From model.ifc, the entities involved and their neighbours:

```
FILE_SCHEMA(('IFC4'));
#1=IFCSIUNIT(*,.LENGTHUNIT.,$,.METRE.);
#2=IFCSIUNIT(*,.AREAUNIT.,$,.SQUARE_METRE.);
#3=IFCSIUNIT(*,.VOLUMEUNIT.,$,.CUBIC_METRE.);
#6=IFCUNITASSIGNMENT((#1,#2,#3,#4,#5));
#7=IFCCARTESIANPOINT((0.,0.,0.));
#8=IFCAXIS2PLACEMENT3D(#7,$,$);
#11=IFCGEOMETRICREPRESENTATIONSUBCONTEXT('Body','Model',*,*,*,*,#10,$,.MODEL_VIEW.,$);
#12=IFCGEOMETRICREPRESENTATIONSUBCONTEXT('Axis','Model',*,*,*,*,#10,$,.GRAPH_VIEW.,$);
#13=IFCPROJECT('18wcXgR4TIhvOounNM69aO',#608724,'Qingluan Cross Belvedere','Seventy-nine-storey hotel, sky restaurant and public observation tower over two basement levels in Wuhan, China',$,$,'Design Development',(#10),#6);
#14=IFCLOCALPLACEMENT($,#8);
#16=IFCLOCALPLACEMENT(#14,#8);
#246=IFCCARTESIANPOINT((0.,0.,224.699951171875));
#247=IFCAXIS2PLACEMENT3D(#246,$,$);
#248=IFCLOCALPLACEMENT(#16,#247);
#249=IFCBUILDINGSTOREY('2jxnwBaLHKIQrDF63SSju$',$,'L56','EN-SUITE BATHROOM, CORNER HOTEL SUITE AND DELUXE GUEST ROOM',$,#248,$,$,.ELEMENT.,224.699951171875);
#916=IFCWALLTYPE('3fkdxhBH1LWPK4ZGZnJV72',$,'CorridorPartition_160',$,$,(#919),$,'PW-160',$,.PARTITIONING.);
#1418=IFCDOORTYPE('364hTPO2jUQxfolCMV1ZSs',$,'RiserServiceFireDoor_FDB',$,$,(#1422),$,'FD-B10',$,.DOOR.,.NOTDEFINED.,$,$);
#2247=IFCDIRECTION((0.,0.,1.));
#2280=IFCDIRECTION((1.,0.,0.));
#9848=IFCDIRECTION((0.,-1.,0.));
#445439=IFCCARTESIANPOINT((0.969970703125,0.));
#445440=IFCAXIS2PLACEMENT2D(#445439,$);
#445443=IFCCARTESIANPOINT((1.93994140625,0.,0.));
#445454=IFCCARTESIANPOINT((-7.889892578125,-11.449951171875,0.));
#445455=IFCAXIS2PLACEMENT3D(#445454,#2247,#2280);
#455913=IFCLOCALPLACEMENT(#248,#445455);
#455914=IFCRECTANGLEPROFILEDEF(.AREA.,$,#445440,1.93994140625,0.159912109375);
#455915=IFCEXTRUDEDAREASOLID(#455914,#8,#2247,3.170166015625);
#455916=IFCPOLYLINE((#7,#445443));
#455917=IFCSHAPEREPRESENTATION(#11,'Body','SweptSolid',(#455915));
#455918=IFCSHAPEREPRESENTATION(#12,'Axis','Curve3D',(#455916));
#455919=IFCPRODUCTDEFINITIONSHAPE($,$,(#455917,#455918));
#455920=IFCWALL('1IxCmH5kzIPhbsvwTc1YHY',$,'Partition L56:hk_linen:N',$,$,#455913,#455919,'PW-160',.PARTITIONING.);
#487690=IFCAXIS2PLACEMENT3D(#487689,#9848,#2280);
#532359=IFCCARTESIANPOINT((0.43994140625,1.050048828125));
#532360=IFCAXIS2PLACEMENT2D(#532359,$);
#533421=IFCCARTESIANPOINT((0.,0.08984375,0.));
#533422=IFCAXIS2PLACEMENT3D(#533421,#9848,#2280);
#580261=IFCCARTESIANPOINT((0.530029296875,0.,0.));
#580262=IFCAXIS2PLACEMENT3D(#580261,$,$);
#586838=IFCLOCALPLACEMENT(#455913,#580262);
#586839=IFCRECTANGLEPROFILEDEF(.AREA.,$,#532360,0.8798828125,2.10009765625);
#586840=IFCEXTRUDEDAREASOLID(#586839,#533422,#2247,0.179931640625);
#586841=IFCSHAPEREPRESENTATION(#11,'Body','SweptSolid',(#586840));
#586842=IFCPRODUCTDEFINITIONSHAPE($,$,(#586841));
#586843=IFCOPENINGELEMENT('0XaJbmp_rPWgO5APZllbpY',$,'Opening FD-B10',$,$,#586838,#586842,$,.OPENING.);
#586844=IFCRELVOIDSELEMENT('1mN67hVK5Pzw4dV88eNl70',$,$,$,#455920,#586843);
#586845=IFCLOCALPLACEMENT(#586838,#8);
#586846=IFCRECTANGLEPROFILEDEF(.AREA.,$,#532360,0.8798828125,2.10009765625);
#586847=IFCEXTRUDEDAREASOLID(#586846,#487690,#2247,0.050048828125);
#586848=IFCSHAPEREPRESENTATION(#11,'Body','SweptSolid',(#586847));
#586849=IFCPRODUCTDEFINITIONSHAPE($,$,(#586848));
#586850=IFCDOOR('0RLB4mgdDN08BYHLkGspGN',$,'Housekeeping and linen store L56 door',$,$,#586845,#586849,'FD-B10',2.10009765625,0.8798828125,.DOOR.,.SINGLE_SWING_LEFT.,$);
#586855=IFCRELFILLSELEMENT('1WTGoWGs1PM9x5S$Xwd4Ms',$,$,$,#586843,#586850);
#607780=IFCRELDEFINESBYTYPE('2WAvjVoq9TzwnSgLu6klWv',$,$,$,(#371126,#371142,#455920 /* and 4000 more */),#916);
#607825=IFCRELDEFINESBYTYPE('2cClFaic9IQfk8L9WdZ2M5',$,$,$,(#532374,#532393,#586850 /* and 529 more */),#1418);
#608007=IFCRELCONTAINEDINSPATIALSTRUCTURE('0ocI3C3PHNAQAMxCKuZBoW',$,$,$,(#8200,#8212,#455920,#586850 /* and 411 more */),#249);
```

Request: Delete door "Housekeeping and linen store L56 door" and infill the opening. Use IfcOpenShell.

```python
import ifcopenshell
import ifcopenshell.api.feature
import ifcopenshell.api.root
import ifcopenshell.geom
import ifcopenshell.util.shape

model = ifcopenshell.open("model.ifc")
settings = ifcopenshell.geom.settings()


def volume(element):
    """Net volume in cubic metres, openings subtracted."""
    shape = ifcopenshell.geom.create_shape(settings, element)
    return ifcopenshell.util.shape.get_volume(shape.geometry)


door = model.by_id(586850)
opening = door.FillsVoids[0].RelatingOpeningElement
wall = opening.VoidsElements[0].RelatingBuildingElement
before = volume(wall)

ifcopenshell.api.root.remove_product(model, product=door)
ifcopenshell.api.feature.remove_feature(model, feature=opening)

after = volume(wall)

print(f"wall volume {before:.3f} -> {after:.3f} m3")

model.write("model-out.ifc")
```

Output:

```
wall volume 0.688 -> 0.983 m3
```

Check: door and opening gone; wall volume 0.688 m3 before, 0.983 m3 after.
